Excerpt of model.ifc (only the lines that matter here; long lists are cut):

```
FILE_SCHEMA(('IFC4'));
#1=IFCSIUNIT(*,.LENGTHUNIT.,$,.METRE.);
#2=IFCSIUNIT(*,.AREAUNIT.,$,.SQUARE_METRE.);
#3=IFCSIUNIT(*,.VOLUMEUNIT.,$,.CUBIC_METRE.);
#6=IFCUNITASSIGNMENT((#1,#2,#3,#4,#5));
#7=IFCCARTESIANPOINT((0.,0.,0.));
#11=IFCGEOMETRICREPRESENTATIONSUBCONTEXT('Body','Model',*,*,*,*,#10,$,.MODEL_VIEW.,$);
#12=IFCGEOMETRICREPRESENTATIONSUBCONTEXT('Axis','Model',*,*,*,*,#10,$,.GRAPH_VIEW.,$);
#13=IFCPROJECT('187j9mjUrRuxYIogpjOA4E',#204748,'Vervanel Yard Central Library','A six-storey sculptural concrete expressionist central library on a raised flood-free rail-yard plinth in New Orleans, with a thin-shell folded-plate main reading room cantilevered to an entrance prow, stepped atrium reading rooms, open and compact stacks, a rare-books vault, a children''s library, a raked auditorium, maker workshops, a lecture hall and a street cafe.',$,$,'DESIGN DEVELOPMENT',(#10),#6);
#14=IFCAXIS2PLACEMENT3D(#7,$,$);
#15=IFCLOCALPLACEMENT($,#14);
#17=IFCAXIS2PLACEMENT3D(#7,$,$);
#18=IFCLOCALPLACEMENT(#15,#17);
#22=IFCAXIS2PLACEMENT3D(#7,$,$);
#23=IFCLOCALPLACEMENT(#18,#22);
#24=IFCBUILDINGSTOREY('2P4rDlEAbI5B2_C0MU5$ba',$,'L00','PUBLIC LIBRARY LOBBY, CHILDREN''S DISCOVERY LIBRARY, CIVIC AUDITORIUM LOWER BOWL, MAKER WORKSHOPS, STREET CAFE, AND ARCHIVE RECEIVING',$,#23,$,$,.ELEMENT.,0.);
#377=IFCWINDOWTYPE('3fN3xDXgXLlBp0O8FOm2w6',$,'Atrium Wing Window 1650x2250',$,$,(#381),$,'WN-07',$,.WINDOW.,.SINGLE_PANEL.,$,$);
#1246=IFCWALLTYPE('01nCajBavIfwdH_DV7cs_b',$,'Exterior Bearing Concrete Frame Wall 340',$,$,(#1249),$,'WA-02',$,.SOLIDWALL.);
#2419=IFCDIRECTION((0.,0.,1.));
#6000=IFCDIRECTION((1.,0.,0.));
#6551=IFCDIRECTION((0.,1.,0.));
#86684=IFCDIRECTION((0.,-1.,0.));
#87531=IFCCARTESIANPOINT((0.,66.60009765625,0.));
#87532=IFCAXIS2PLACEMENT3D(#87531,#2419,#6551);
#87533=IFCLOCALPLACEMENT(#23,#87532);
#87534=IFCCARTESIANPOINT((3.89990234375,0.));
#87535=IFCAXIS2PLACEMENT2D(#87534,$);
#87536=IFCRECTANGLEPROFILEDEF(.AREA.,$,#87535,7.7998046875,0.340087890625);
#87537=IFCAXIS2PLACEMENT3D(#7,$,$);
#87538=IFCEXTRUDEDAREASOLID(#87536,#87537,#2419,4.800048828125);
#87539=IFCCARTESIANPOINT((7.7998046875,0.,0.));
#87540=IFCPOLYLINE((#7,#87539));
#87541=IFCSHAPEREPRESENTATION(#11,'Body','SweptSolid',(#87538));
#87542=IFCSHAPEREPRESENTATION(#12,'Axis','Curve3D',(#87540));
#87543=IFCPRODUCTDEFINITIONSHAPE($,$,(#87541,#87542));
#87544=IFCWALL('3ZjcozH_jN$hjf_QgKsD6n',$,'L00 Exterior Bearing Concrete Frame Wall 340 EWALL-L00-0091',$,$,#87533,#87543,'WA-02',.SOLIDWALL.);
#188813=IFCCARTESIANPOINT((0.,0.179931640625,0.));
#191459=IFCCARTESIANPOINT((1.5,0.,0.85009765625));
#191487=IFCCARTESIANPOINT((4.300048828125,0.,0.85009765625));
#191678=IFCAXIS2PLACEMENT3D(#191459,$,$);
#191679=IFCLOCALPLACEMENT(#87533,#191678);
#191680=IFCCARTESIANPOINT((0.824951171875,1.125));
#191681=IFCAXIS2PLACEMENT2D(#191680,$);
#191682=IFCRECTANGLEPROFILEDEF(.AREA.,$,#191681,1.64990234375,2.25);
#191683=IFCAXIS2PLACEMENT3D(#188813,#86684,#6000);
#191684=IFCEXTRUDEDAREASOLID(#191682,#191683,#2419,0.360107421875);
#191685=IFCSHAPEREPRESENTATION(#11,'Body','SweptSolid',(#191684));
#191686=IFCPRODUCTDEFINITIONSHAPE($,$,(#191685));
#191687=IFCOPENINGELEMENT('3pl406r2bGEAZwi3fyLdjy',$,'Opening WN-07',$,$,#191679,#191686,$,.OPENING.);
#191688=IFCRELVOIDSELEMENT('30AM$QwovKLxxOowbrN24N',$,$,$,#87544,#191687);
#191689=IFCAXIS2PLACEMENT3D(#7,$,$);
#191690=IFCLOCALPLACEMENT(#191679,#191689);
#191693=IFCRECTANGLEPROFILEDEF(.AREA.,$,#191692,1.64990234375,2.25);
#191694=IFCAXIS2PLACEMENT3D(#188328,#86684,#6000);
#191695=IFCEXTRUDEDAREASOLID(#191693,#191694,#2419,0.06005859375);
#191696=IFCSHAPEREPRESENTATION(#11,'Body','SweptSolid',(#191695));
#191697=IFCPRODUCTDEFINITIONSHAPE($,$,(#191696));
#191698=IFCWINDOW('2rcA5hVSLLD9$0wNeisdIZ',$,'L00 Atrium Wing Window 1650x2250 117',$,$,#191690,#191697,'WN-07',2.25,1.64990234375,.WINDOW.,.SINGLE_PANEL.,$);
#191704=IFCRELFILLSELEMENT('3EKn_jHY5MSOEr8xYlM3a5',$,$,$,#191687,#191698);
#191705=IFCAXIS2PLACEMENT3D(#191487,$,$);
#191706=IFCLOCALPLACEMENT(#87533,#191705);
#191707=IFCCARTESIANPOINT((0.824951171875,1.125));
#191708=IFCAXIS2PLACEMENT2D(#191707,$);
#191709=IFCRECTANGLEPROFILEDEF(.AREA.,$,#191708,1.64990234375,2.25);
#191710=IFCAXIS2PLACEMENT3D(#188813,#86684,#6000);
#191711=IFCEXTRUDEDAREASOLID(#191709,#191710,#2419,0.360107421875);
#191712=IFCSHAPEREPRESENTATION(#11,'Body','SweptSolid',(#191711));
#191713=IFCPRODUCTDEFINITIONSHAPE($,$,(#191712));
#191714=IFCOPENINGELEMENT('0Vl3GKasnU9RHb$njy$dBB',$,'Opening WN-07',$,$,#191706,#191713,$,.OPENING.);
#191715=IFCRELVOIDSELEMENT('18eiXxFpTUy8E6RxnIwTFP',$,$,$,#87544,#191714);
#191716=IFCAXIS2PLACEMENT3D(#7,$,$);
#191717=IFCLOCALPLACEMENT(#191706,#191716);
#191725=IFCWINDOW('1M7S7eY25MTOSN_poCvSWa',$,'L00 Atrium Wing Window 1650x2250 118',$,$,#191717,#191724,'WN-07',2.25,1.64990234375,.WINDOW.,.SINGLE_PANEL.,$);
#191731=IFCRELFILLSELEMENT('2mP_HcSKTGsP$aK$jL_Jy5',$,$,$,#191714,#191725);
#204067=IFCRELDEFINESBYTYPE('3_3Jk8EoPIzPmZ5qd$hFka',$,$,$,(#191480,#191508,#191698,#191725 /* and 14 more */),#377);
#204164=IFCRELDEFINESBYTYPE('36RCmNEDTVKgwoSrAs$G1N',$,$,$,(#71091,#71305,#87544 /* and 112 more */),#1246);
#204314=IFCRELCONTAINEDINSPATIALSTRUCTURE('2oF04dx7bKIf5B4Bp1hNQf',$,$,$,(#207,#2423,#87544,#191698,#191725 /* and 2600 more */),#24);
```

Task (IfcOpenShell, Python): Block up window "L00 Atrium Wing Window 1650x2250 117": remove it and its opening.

```python
import ifcopenshell
import ifcopenshell.api.feature
import ifcopenshell.api.root
import ifcopenshell.geom
import ifcopenshell.util.shape

model = ifcopenshell.open("model.ifc")
settings = ifcopenshell.geom.settings()


def volume(element):
    """Net volume in cubic metres, openings subtracted."""
    shape = ifcopenshell.geom.create_shape(settings, element)
    return ifcopenshell.util.shape.get_volume(shape.geometry)


window = model.by_id(191698)
opening = window.FillsVoids[0].RelatingOpeningElement
wall = opening.VoidsElements[0].RelatingBuildingElement
before = volume(wall)

ifcopenshell.api.root.remove_product(model, product=window)
ifcopenshell.api.feature.remove_feature(model, feature=opening)

after = volume(wall)

print(f"wall volume {before:.3f} -> {after:.3f} m3")

model.write("model_updated.ifc")
```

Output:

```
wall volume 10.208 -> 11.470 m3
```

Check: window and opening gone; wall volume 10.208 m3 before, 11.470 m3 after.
